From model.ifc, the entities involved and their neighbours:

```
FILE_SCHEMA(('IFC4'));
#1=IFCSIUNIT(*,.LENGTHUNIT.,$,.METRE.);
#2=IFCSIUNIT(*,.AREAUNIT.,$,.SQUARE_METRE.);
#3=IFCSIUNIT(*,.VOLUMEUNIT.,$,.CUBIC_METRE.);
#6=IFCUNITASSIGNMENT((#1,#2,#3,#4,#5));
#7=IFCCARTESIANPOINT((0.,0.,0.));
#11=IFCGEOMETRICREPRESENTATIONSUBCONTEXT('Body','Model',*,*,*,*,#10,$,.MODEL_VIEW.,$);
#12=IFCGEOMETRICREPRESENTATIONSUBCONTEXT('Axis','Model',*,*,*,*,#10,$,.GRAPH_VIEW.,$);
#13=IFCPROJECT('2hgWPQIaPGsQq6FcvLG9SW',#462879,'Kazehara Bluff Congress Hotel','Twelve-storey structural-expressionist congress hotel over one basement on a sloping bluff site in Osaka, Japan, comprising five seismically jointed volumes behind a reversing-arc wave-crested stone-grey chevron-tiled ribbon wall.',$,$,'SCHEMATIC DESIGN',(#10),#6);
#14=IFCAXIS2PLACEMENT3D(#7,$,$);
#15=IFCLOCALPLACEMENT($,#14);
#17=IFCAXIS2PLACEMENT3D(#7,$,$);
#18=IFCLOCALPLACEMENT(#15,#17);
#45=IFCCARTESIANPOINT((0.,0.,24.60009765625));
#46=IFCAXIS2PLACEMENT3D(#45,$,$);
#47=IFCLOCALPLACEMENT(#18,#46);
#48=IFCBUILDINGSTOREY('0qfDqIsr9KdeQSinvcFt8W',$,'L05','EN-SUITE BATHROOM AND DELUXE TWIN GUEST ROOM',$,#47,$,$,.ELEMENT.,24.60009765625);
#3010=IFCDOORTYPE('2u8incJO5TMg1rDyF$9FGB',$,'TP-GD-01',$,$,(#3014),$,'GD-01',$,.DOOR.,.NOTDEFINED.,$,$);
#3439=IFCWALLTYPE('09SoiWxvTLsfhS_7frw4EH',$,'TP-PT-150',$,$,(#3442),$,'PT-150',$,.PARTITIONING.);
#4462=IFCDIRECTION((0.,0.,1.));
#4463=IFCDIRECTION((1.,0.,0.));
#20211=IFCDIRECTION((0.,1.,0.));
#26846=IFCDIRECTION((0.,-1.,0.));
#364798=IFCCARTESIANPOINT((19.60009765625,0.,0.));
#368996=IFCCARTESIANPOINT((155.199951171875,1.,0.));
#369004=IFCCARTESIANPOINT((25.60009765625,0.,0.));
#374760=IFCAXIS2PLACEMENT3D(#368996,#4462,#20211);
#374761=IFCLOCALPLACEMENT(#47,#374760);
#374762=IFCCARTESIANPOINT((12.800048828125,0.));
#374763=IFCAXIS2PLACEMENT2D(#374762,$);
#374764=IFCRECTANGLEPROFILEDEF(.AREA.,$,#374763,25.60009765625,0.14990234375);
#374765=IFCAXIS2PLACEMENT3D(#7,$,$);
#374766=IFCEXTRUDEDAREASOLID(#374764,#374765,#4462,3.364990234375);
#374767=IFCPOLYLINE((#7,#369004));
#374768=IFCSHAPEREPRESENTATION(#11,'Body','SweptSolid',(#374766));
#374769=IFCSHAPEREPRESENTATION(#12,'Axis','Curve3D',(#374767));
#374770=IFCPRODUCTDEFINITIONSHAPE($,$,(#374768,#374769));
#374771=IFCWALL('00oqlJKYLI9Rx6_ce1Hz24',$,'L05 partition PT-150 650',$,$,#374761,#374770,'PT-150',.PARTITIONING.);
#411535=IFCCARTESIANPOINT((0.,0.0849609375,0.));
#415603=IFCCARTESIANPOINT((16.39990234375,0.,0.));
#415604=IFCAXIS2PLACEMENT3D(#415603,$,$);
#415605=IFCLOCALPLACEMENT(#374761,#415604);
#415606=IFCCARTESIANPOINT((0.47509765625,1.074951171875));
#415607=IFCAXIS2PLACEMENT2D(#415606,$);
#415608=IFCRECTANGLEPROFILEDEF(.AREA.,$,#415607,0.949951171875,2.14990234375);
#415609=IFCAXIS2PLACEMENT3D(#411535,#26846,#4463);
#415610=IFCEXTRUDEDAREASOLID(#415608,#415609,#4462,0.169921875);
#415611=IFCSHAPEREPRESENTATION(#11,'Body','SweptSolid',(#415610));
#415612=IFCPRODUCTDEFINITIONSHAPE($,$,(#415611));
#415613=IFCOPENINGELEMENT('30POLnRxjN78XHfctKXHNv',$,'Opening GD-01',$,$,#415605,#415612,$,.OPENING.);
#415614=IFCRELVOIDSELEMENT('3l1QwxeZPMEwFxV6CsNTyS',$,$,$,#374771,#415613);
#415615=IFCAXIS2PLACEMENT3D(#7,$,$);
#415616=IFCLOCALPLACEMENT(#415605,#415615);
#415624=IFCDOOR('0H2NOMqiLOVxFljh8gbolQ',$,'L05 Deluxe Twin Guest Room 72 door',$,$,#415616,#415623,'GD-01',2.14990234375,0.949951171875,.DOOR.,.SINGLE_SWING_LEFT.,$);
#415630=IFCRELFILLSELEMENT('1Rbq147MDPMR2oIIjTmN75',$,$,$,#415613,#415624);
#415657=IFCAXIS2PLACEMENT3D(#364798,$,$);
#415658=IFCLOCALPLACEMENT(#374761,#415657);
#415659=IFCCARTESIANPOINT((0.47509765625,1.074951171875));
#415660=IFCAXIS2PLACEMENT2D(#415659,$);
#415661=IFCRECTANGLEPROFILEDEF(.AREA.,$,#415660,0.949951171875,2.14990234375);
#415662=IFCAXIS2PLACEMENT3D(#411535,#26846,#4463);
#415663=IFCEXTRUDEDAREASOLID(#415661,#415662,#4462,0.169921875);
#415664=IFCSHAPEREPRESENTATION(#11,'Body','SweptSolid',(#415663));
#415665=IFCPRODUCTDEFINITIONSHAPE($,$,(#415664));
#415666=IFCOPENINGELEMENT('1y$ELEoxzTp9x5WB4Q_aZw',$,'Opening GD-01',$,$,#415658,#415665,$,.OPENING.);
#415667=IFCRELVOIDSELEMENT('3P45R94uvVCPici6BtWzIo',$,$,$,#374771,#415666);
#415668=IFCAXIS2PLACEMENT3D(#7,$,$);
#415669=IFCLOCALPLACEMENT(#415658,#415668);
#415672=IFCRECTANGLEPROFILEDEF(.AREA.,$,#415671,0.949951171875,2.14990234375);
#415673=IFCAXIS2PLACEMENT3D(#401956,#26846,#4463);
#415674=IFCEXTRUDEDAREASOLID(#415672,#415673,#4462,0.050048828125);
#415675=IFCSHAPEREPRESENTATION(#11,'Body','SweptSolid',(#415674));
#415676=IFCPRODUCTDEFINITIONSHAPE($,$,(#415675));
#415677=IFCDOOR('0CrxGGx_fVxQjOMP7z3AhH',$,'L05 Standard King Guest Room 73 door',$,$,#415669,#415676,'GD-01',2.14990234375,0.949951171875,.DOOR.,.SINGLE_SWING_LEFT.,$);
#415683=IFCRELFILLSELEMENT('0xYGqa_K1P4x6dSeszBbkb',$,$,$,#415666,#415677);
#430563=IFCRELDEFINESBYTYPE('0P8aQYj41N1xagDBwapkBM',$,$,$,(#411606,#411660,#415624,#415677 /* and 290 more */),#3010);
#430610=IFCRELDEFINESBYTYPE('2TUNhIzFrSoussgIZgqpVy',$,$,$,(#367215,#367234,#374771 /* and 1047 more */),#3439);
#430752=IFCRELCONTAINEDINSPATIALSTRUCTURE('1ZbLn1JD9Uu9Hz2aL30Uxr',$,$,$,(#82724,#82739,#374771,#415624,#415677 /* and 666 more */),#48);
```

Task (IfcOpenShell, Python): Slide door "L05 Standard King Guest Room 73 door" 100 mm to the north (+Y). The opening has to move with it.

```python
import ifcopenshell
import ifcopenshell.api.geometry
import ifcopenshell.util.placement
import ifcopenshell.util.unit

model = ifcopenshell.open("model.ifc")
unit_scale = ifcopenshell.util.unit.calculate_unit_scale(model)

door = model.by_guid("0CrxGGx_fVxQjOMP7z3AhH")
opening = door.FillsVoids[0].RelatingOpeningElement
wall = opening.VoidsElements[0].RelatingBuildingElement

wall_matrix = ifcopenshell.util.placement.get_local_placement(wall.ObjectPlacement)
shift = wall_matrix[:3, 0] * 0.1 / unit_scale
before = ifcopenshell.util.placement.get_local_placement(door.ObjectPlacement)[:3, 3].copy()

# The door is placed relative to its opening, so it follows when the opening moves.
matrix = ifcopenshell.util.placement.get_local_placement(opening.ObjectPlacement)
matrix[:3, 3] += shift
ifcopenshell.api.geometry.edit_object_placement(
    model, product=opening, matrix=matrix, is_si=False, should_transform_children=True
)

after = ifcopenshell.util.placement.get_local_placement(door.ObjectPlacement)[:3, 3]
print("door moved by", (after - before).round(3) + 0.0)

model.write("model_updated.ifc")
```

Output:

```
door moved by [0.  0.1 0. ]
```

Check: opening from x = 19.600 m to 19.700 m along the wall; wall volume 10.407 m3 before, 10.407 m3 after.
